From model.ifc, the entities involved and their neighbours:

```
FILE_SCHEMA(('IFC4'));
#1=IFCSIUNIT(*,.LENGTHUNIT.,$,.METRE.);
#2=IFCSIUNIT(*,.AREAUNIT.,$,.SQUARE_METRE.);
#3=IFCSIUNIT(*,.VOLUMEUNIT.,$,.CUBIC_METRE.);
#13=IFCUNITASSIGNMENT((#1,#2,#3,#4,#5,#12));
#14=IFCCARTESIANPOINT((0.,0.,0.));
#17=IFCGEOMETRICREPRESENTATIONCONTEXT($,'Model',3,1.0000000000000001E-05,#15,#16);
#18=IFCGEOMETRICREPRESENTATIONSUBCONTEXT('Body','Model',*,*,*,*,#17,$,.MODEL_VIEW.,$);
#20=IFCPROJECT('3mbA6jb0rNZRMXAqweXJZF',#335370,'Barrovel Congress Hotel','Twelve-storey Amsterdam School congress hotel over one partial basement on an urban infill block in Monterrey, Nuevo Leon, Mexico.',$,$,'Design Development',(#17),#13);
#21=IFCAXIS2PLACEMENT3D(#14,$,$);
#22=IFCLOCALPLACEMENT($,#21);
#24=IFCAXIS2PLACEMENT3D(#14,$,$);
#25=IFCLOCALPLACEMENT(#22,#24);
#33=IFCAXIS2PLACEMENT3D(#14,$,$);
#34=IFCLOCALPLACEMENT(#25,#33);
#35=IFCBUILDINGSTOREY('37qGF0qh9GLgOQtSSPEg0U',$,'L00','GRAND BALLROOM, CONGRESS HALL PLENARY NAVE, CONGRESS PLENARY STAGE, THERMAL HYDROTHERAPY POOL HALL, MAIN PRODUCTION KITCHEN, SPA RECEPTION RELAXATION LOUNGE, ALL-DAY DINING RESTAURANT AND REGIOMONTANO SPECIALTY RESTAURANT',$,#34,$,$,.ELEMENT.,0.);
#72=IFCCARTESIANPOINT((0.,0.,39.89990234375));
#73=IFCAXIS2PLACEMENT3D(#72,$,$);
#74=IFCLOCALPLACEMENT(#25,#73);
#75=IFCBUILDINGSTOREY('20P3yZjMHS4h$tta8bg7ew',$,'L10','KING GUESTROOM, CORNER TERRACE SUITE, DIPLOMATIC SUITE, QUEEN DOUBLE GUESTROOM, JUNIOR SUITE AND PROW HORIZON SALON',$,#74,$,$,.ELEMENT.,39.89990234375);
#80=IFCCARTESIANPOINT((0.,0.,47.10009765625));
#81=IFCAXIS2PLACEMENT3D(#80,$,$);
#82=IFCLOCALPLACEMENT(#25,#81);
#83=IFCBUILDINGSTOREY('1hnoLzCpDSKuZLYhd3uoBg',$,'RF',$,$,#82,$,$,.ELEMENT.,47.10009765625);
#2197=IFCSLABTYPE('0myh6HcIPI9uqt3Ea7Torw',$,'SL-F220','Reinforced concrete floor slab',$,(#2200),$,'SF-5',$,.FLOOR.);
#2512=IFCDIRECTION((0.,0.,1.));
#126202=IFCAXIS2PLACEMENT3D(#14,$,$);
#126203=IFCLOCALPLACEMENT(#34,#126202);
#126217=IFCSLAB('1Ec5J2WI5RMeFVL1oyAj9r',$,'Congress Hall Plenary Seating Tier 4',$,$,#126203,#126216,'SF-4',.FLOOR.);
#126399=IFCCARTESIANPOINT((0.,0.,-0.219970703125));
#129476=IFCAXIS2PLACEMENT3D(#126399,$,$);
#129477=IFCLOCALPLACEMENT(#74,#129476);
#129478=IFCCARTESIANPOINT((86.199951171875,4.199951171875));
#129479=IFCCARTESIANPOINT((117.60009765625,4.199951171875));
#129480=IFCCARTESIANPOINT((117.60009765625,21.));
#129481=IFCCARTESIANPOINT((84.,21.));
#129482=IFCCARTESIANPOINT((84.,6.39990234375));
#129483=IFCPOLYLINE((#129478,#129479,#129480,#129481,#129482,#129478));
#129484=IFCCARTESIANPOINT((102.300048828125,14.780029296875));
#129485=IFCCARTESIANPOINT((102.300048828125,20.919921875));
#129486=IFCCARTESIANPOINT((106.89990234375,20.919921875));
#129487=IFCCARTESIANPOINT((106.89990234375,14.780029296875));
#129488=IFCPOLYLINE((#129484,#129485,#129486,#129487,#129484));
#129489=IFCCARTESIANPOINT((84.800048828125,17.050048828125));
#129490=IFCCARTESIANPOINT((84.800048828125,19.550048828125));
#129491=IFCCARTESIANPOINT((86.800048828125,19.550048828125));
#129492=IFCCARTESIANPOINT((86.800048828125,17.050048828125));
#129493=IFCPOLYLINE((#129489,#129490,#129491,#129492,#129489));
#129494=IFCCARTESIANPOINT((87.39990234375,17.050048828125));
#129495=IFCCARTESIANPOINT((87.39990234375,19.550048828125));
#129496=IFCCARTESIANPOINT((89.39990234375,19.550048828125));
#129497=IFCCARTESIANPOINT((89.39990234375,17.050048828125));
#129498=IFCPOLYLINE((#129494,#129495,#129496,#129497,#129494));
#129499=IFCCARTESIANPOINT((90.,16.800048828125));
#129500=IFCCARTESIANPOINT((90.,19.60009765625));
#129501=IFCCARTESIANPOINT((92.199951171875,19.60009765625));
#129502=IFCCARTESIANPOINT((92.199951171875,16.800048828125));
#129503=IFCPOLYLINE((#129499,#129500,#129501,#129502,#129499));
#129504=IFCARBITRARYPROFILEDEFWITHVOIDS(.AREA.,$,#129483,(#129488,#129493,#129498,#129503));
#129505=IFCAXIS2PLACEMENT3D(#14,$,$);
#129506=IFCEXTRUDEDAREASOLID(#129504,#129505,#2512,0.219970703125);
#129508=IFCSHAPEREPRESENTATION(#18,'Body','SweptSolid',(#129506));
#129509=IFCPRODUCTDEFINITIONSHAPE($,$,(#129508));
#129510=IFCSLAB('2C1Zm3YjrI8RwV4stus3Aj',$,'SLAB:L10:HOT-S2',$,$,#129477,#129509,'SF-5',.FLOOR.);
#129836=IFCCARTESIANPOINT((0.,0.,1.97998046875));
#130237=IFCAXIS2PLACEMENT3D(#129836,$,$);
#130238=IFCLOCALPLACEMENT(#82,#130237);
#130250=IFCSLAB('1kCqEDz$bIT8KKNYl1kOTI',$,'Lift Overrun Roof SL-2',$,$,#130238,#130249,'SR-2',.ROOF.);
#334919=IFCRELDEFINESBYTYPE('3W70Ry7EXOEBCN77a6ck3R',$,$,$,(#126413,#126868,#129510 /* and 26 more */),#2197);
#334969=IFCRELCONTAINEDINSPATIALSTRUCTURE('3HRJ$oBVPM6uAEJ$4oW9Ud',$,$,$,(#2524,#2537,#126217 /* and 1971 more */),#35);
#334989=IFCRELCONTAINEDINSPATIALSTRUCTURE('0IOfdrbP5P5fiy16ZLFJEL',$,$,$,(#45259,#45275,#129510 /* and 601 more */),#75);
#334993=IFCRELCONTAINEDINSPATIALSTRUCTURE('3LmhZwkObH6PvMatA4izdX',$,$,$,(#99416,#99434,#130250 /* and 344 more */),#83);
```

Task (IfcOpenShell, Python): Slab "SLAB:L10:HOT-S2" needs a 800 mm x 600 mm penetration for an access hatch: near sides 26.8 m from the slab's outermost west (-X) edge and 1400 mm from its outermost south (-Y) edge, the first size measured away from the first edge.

```python
import numpy as np
import ifcopenshell
import ifcopenshell.api.feature
import ifcopenshell.api.geometry
import ifcopenshell.api.root
import ifcopenshell.geom
import ifcopenshell.util.placement
import ifcopenshell.util.representation
import ifcopenshell.util.shape
import ifcopenshell.util.unit

model = ifcopenshell.open("model.ifc")
unit_scale = ifcopenshell.util.unit.calculate_unit_scale(model)
settings = ifcopenshell.geom.settings()


def volume(element):
    """Net volume in cubic metres, openings subtracted."""
    shape = ifcopenshell.geom.create_shape(settings, element)
    return ifcopenshell.util.shape.get_volume(shape.geometry)


slab = model.by_guid("2C1Zm3YjrI8RwV4stus3Aj")
before = volume(slab)

# Extent in the slab's own axes, in metres. The edges named are its -X and -Y sides.
slab_shape = ifcopenshell.geom.create_shape(settings, slab)
vertices = ifcopenshell.util.shape.get_vertices(slab_shape.geometry)
x_min, y_min, bottom = vertices.min(axis=0)
top = vertices[:, 2].max()

opening = ifcopenshell.api.root.create_entity(model, ifc_class="IfcOpeningElement", name="Access hatch opening", predefined_type="OPENING")
context = ifcopenshell.util.representation.get_context(model, "Model", "Body", "MODEL_VIEW")
width, depth = 0.8, 0.6
outline = [(0.0, 0.0), (width, 0.0), (width, depth), (0.0, depth), (0.0, 0.0)]
# Overshoot both faces by 50 mm so the cut is clean.
shape = ifcopenshell.api.geometry.add_slab_representation(
    model, context=context, depth=top - bottom + 0.1, polyline=outline
)
ifcopenshell.api.geometry.assign_representation(model, product=opening, representation=shape)

matrix = ifcopenshell.util.placement.get_local_placement(slab.ObjectPlacement)
matrix[:, 3] = matrix @ np.append(np.array([x_min + 26.8, y_min + 1.4, bottom - 0.05]) / unit_scale, 1.0)
ifcopenshell.api.geometry.edit_object_placement(model, product=opening, matrix=matrix, is_si=False)
ifcopenshell.api.feature.add_feature(model, feature=opening, element=slab)

after = volume(slab)

print(f"slab volume {before:.3f} -> {after:.3f} m3")

model.write("model_rev.ifc")
```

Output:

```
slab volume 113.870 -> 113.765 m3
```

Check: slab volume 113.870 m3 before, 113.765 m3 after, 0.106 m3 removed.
